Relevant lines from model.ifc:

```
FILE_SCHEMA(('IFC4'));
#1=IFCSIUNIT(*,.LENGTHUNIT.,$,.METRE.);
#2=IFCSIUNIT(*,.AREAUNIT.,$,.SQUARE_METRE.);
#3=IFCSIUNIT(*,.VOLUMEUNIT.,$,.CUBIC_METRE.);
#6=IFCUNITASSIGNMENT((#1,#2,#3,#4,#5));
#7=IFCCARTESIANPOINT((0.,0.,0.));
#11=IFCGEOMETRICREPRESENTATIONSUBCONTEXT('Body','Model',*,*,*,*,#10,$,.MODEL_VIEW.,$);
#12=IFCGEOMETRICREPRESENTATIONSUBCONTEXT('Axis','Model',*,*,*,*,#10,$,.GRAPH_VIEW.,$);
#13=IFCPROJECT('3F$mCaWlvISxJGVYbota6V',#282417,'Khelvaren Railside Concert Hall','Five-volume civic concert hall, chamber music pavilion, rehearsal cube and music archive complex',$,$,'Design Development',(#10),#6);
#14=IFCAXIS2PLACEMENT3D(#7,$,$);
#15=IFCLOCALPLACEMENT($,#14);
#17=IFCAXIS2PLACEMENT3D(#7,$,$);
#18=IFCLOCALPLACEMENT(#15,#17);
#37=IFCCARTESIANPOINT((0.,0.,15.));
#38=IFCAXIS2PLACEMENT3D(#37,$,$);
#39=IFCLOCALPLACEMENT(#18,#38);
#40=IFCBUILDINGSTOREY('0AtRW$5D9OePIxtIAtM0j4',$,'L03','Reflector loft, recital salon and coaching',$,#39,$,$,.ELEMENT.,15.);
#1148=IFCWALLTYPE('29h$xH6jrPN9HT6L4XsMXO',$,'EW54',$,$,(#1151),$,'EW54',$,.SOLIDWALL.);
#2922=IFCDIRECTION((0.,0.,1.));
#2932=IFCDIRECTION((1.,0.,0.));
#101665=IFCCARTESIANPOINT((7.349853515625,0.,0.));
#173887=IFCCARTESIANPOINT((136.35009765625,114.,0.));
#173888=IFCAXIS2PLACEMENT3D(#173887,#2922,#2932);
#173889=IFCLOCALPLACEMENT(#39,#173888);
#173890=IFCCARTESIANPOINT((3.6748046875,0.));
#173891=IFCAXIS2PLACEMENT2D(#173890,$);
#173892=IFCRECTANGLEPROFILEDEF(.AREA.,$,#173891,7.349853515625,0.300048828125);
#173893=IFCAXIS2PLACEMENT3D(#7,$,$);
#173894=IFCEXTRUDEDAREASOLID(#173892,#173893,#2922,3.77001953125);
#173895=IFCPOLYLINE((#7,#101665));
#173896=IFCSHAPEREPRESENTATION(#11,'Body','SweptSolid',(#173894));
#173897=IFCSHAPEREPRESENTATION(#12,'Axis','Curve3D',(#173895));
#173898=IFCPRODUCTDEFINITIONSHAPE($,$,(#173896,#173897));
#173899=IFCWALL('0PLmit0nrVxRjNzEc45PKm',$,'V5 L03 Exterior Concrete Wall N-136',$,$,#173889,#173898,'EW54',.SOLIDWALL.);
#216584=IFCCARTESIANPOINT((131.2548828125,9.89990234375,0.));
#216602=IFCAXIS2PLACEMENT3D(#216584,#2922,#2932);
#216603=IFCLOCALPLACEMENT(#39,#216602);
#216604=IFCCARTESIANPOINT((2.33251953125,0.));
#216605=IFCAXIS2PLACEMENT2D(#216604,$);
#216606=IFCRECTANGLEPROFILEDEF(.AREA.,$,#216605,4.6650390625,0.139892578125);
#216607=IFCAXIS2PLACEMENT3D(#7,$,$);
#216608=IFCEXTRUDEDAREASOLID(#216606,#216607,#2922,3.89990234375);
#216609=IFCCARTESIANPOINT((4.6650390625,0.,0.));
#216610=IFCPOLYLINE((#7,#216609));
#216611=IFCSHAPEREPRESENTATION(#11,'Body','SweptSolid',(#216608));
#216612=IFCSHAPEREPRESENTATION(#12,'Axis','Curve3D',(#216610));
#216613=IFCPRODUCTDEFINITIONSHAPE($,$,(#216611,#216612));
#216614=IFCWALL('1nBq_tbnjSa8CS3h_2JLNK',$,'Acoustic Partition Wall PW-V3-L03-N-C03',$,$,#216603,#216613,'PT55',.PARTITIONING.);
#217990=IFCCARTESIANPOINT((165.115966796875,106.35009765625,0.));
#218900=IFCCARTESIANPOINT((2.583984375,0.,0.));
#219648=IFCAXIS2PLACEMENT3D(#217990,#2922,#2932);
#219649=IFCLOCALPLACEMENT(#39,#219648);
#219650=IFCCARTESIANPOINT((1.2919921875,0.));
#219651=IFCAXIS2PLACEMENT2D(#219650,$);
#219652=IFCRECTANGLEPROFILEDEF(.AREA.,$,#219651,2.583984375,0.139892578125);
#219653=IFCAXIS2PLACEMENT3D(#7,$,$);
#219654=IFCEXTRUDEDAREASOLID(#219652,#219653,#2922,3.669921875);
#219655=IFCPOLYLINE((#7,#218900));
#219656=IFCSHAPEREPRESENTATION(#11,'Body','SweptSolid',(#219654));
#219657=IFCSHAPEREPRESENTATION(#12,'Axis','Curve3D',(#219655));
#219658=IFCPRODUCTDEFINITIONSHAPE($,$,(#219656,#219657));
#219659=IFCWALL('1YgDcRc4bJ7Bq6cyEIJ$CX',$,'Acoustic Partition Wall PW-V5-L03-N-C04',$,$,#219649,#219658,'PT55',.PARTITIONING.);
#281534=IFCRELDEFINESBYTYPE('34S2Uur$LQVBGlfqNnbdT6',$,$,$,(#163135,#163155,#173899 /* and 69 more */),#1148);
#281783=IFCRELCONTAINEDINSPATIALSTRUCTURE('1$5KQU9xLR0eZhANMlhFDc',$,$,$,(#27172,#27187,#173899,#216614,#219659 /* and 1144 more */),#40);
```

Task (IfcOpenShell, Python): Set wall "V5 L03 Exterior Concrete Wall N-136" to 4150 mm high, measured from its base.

```python
import ifcopenshell
import ifcopenshell.geom
import ifcopenshell.util.representation
import ifcopenshell.util.shape
import ifcopenshell.util.unit

model = ifcopenshell.open("model.ifc")
unit_scale = ifcopenshell.util.unit.calculate_unit_scale(model)
settings = ifcopenshell.geom.settings()


def volume(element):
    """Net volume in cubic metres, openings subtracted."""
    shape = ifcopenshell.geom.create_shape(settings, element)
    return ifcopenshell.util.shape.get_volume(shape.geometry)


wall = model.by_guid("0PLmit0nrVxRjNzEc45PKm")
before = volume(wall)

body = ifcopenshell.util.representation.get_representation(wall, "Model", "Body")
solid = body.Items[0]
old_height = solid.Depth
solid.Depth = 4.15 / unit_scale
after = volume(wall)

print(f"height {old_height:g} -> {solid.Depth:g}, volume {before:.3f} -> {after:.3f} m3")

model.write("model_v2.ifc")
```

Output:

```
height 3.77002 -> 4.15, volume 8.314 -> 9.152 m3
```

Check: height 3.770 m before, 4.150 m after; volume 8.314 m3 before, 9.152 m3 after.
